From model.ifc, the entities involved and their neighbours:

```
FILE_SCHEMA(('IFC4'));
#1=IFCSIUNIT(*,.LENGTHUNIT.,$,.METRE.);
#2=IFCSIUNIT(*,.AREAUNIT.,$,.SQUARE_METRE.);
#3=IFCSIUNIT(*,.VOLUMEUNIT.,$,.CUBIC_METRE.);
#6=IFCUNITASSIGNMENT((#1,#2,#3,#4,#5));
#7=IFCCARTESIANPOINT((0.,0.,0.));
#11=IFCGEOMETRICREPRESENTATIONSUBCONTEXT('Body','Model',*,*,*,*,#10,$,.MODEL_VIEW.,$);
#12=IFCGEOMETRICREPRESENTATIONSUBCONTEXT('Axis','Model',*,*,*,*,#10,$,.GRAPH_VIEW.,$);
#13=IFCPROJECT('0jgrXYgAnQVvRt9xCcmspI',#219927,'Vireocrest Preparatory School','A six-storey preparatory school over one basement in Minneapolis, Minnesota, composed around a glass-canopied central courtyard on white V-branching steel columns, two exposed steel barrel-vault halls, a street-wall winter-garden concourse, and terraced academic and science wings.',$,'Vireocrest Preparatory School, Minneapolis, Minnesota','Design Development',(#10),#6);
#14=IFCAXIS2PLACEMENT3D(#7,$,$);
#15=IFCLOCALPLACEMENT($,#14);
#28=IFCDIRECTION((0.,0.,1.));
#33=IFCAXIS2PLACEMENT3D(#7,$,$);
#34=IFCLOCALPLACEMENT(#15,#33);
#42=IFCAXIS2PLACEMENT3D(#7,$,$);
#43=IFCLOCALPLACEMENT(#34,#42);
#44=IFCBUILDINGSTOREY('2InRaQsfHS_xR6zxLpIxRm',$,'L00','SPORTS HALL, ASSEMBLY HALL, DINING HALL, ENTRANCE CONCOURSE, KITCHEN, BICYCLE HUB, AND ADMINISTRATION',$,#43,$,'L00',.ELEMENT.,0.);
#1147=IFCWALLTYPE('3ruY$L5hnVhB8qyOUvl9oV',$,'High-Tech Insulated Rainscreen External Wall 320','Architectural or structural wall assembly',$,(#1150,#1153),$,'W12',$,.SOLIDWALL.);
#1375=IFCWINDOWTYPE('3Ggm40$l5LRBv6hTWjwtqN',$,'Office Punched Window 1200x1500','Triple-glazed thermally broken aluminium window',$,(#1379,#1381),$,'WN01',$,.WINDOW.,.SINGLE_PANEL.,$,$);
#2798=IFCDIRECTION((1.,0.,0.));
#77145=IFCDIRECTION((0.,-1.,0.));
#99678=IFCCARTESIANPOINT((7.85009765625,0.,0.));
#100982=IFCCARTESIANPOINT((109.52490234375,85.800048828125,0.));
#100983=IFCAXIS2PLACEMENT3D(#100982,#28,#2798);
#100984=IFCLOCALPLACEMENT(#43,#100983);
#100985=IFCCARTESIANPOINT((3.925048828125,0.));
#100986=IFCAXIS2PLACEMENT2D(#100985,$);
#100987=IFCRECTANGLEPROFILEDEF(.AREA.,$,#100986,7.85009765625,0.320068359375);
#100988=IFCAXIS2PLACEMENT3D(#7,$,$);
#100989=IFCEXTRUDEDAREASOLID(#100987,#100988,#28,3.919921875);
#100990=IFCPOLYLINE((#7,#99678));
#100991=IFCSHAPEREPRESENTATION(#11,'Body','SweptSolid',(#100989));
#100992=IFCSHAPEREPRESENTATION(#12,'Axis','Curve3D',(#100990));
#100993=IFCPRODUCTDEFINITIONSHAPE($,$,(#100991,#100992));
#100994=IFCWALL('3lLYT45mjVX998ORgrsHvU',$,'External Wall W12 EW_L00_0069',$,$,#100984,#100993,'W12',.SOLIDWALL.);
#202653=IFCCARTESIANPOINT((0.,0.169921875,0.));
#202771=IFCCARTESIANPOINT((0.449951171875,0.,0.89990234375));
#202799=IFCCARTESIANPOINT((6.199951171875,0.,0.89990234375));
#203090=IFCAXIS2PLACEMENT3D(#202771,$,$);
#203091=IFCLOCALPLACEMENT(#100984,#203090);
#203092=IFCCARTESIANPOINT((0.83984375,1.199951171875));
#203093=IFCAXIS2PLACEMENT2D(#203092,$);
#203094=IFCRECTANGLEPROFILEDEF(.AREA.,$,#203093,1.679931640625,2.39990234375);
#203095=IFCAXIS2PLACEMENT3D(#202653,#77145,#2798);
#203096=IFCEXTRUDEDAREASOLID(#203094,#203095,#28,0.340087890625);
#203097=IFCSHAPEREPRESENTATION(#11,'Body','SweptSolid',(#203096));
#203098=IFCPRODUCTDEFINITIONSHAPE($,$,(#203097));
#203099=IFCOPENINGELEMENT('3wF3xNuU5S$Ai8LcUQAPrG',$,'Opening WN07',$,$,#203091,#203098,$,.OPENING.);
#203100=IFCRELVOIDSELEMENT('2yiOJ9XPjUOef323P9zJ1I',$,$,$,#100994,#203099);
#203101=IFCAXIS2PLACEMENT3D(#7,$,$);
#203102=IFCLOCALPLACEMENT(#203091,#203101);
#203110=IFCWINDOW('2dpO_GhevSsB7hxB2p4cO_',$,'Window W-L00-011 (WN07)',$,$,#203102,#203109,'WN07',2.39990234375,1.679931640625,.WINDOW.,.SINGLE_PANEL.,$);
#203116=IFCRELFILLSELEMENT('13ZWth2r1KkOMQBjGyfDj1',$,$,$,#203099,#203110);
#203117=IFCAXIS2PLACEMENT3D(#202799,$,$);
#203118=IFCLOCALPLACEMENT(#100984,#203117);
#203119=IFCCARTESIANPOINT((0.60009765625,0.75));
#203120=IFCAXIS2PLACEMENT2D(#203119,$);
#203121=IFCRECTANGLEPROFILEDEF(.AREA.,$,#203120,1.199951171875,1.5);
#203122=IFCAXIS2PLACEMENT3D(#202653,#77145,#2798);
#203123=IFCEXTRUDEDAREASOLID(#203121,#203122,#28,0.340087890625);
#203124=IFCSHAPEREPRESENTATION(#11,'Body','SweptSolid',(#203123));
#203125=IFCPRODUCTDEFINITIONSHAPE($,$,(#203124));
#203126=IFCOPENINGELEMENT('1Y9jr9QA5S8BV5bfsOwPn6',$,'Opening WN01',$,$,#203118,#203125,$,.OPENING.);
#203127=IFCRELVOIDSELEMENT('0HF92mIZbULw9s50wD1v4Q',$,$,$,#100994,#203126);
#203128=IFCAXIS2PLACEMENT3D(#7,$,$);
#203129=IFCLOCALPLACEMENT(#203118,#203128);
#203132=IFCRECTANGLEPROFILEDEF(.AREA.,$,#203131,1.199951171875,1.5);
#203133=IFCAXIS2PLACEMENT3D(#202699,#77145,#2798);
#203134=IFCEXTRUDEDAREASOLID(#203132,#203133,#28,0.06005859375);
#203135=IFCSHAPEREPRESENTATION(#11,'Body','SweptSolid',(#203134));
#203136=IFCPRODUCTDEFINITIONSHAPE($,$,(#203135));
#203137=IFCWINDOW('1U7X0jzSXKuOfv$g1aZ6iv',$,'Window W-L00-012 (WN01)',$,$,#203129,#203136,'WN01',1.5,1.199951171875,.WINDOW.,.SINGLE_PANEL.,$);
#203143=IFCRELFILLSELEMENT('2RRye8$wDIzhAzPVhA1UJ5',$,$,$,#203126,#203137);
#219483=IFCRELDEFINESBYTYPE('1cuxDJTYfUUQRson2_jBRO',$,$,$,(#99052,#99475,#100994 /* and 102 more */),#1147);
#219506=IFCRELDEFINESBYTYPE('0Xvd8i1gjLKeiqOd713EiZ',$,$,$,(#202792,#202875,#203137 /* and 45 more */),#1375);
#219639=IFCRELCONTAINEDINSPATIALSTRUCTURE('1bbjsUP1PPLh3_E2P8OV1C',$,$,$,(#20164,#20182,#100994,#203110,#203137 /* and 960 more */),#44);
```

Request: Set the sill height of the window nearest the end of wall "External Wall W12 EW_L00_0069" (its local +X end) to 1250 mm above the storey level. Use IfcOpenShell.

```python
import numpy as np
import ifcopenshell
import ifcopenshell.api.geometry
import ifcopenshell.geom
import ifcopenshell.util.element
import ifcopenshell.util.placement
import ifcopenshell.util.shape
import ifcopenshell.util.unit

model = ifcopenshell.open("model.ifc")
unit_scale = ifcopenshell.util.unit.calculate_unit_scale(model)

window = model.by_guid("1U7X0jzSXKuOfv$g1aZ6iv")
opening = window.FillsVoids[0].RelatingOpeningElement
storey = ifcopenshell.util.element.get_container(window, ifc_class="IfcBuildingStorey")
level = ifcopenshell.util.placement.get_local_placement(storey.ObjectPlacement)[2, 3]

# The opening's origin need not be at the sill, so measure its lowest point.
shape = ifcopenshell.geom.create_shape(ifcopenshell.geom.settings(), opening)
bottom = ifcopenshell.util.shape.get_shape_bottom_elevation(shape, shape.geometry) / unit_scale
dz = level + 1.25 - bottom

shift = np.array([0.0, 0.0, dz])
# The window is placed relative to its opening, so it follows when the opening moves.
matrix = ifcopenshell.util.placement.get_local_placement(opening.ObjectPlacement)
matrix[:3, 3] += shift
ifcopenshell.api.geometry.edit_object_placement(
    model, product=opening, matrix=matrix, is_si=False, should_transform_children=True
)

print(f"moved by {dz * unit_scale:+.3f} m")

model.write("model-out.ifc")
```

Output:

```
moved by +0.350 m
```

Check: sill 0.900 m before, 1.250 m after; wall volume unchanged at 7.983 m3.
